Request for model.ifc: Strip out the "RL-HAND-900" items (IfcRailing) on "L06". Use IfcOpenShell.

First a look at what the model holds.

```python
import ifcopenshell
import ifcopenshell.util.element

model = ifcopenshell.open("model.ifc")
print(model.schema)
storey = next(s for s in model.by_type("IfcBuildingStorey") if s.Name == "L06")
railings = [e for e in ifcopenshell.util.element.get_decomposition(storey) if e.is_a("IfcRailing")]
seen = {}
for e in railings:
    element_type = ifcopenshell.util.element.get_type(e)
    name = element_type.Name if element_type not in (None, e) else None
    seen[name] = seen.get(name, 0) + 1
for name, count in sorted(seen.items(), key=str):
    print(count, "x", name)
```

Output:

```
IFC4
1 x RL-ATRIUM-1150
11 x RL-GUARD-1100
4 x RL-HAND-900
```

```python
import ifcopenshell
import ifcopenshell.api.root
import ifcopenshell.util.element

model = ifcopenshell.open("model.ifc")

storey = next(s for s in model.by_type("IfcBuildingStorey") if s.Name == "L06")
railings = [e for e in ifcopenshell.util.element.get_decomposition(storey) if e.is_a("IfcRailing")]
targets = [e for e in railings if (t := ifcopenshell.util.element.get_type(e)) not in (None, e) and t.Name == "RL-HAND-900"]

for e in targets:
    ifcopenshell.api.root.remove_product(model, product=e)
print(len(targets), "removed")

model.write("model_edited.ifc")
```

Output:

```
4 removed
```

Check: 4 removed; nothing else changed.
